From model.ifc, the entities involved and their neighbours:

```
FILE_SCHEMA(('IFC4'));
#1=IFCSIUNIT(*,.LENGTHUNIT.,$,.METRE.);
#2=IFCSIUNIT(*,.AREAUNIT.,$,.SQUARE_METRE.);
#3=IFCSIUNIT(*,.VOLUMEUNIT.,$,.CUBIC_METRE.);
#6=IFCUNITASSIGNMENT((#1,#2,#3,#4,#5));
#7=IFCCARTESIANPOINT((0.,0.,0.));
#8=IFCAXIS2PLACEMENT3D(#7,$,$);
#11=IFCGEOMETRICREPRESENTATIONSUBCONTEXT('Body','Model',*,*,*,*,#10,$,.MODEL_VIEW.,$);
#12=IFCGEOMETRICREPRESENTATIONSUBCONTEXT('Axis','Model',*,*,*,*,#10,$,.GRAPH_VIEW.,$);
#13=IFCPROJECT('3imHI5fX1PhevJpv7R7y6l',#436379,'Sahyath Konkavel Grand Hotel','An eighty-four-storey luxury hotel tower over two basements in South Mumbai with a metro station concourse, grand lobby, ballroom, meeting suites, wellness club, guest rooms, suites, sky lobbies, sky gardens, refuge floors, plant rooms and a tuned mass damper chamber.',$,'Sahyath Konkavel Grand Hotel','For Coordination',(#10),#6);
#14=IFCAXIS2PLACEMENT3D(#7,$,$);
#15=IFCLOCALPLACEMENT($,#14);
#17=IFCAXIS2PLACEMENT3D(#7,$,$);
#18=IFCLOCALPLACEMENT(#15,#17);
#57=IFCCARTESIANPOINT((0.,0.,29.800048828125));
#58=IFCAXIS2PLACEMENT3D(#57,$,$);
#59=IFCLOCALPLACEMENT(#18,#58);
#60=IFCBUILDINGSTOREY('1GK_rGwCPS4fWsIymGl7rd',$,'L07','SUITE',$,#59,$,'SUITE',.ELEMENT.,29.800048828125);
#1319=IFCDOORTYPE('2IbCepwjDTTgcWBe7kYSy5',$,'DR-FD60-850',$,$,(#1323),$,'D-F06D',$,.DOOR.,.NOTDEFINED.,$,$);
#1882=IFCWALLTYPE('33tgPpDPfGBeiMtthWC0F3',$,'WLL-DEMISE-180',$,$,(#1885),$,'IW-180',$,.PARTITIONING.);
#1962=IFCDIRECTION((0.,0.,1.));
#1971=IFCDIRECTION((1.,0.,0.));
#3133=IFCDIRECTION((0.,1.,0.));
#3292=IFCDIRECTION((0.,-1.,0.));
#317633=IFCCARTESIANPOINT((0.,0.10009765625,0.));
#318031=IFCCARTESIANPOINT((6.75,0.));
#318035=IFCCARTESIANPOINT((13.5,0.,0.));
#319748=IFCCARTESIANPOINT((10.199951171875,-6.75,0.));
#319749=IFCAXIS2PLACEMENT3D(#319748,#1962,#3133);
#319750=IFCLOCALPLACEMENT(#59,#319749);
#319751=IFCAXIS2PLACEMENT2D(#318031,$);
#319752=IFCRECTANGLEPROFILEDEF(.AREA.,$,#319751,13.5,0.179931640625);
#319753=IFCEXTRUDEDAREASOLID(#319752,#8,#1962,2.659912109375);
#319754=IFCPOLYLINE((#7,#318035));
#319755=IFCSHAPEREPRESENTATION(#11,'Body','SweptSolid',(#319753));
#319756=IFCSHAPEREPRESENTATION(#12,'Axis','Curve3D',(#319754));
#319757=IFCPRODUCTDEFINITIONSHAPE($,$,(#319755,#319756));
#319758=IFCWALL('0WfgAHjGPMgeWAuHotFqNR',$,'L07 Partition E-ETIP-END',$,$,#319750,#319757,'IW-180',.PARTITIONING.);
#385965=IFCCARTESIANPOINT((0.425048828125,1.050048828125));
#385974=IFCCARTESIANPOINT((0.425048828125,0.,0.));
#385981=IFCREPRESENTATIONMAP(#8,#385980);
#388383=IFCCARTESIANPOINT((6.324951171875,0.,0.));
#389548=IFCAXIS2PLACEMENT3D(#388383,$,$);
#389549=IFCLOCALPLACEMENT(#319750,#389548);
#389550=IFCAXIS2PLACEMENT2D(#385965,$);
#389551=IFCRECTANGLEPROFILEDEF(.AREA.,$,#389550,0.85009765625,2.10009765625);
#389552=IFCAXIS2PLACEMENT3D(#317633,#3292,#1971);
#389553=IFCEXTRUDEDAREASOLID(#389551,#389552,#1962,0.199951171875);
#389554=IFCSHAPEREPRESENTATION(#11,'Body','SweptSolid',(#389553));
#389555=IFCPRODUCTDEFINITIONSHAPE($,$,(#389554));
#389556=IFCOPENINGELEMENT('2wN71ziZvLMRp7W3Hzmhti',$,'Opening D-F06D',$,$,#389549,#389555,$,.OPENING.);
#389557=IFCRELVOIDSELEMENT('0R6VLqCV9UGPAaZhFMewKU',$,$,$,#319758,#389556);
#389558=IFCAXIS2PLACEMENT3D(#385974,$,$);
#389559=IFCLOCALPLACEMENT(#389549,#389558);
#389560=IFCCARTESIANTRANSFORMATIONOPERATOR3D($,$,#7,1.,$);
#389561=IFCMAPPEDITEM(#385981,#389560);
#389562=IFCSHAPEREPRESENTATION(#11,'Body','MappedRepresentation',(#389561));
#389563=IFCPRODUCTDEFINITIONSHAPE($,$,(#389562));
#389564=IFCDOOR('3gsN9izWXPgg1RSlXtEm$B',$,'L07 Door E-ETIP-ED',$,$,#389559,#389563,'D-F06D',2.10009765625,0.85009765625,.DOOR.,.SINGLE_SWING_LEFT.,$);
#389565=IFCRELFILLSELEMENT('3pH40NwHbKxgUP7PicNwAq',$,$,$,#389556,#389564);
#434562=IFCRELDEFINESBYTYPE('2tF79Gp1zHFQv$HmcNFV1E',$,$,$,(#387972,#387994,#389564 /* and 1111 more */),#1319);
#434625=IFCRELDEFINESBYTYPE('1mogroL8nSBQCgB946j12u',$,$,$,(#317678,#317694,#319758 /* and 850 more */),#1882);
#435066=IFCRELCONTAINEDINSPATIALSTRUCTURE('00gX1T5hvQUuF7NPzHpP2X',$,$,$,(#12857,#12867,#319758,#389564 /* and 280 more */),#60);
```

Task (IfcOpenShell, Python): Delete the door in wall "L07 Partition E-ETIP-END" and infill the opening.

```python
import ifcopenshell
import ifcopenshell.api.feature
import ifcopenshell.api.root
import ifcopenshell.geom
import ifcopenshell.util.shape

model = ifcopenshell.open("model.ifc")
settings = ifcopenshell.geom.settings()


def volume(element):
    """Net volume in cubic metres, openings subtracted."""
    shape = ifcopenshell.geom.create_shape(settings, element)
    return ifcopenshell.util.shape.get_volume(shape.geometry)


door = model.by_id(389564)
opening = door.FillsVoids[0].RelatingOpeningElement
wall = opening.VoidsElements[0].RelatingBuildingElement
before = volume(wall)

ifcopenshell.api.root.remove_product(model, product=door)
ifcopenshell.api.feature.remove_feature(model, feature=opening)

after = volume(wall)

print(f"wall volume {before:.3f} -> {after:.3f} m3")

model.write("model-out.ifc")
```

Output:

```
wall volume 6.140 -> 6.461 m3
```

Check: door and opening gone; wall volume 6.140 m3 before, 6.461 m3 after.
